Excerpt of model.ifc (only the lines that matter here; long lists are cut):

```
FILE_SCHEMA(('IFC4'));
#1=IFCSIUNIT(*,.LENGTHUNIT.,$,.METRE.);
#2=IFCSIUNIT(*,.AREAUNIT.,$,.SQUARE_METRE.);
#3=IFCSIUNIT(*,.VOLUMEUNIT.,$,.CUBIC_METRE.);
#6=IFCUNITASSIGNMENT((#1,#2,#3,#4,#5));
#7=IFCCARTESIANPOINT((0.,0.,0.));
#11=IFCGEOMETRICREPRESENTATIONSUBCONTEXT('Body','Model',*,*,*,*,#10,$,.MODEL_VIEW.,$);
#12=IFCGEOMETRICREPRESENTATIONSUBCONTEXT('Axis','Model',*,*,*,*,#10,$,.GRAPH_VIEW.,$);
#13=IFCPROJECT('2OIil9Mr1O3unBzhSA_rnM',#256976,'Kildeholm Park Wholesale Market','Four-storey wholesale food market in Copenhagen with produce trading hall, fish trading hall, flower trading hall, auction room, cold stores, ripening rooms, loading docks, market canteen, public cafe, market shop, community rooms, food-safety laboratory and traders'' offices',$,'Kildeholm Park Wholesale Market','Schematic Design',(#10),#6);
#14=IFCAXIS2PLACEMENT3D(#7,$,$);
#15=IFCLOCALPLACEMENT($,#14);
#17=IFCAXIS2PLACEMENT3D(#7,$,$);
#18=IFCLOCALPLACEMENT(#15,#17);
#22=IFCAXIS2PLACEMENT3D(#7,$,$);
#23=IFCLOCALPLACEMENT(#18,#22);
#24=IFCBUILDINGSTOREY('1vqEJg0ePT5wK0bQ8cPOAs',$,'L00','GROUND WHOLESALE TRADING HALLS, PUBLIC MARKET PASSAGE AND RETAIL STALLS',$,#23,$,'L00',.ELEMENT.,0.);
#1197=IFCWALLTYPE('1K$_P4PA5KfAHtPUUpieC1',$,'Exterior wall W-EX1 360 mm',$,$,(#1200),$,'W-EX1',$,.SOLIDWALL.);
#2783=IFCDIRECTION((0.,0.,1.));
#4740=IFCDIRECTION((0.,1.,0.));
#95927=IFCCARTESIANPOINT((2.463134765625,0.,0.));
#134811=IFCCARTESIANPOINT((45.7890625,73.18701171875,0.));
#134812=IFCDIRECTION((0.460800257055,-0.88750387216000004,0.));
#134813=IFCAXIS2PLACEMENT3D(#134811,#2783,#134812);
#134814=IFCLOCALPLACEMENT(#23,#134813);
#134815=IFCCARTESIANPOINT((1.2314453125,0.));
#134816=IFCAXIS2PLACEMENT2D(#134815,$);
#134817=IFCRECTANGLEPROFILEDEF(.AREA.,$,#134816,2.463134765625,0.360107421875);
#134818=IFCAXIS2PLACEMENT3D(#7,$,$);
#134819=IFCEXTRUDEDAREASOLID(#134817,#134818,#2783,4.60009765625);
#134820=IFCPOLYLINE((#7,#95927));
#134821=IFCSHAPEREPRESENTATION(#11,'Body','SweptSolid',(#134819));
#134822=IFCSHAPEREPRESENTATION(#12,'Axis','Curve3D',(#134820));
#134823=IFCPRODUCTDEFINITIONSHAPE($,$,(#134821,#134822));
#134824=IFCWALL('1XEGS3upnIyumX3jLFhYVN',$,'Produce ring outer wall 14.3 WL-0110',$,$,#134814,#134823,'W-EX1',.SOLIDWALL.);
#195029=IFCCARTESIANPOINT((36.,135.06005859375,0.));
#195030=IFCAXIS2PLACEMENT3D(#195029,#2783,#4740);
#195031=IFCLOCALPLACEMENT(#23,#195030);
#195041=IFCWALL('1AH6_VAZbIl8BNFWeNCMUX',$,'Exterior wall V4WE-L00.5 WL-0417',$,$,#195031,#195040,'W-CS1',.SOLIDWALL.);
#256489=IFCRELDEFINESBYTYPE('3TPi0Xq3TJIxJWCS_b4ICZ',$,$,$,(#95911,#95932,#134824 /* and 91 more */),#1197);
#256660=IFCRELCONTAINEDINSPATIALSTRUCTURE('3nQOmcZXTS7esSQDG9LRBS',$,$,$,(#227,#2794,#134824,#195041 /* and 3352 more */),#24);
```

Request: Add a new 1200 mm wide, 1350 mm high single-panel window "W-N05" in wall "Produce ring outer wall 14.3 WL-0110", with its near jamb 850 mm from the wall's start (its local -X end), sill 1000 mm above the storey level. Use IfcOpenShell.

```python
import numpy as np
import ifcopenshell
import ifcopenshell.api.feature
import ifcopenshell.api.geometry
import ifcopenshell.api.root
import ifcopenshell.api.spatial
import ifcopenshell.geom
import ifcopenshell.util.element
import ifcopenshell.util.placement
import ifcopenshell.util.representation
import ifcopenshell.util.shape
import ifcopenshell.util.unit

model = ifcopenshell.open("model.ifc")
unit_scale = ifcopenshell.util.unit.calculate_unit_scale(model)
settings = ifcopenshell.geom.settings()


def volume(element):
    """Net volume in cubic metres, openings subtracted."""
    shape = ifcopenshell.geom.create_shape(settings, element)
    return ifcopenshell.util.shape.get_volume(shape.geometry)


wall = model.by_guid("1XEGS3upnIyumX3jLFhYVN")
storey = ifcopenshell.util.element.get_container(wall, ifc_class="IfcBuildingStorey")
context = ifcopenshell.util.representation.get_context(model, "Model", "Body", "MODEL_VIEW")
before = volume(wall)

width, height, from_end, sill = 1.2, 1.35, 0.85, 1  # metres

# The wall runs along its own X axis, and the end named is its -X end.
wall_shape = ifcopenshell.geom.create_shape(settings, wall)
x, y, z = ifcopenshell.util.shape.get_vertices(wall_shape.geometry).T
start = x.min() + from_end
face, thickness = float(y.min()), float(y.max() - y.min())
wall_matrix = ifcopenshell.util.placement.get_local_placement(wall.ObjectPlacement)
level = ifcopenshell.util.placement.get_local_placement(storey.ObjectPlacement)[2, 3]


def in_wall(x, y):
    """Placement at x, y metres in the wall's axes, at sill height."""
    matrix = wall_matrix.copy()
    matrix[:, 3] = wall_matrix @ np.array([x / unit_scale, y / unit_scale, 0.0, 1.0])
    matrix[2, 3] = level + sill / unit_scale
    return matrix


# Opening: a box that overshoots both wall faces by 50 mm.
opening = ifcopenshell.api.root.create_entity(model, ifc_class="IfcOpeningElement", predefined_type="OPENING")
box = ifcopenshell.api.geometry.add_wall_representation(
    model, context=context, length=width, height=height, thickness=thickness + 0.1
)
ifcopenshell.api.geometry.assign_representation(model, product=opening, representation=box)
ifcopenshell.api.geometry.edit_object_placement(model, product=opening, matrix=in_wall(start, face - 0.05), is_si=False)
ifcopenshell.api.feature.add_feature(model, feature=opening, element=wall)

window = ifcopenshell.api.root.create_entity(model, ifc_class="IfcWindow", name="W-N05", predefined_type="WINDOW")
window.OverallWidth, window.OverallHeight = width / unit_scale, height / unit_scale
window.PartitioningType = "SINGLE_PANEL"
body = ifcopenshell.api.geometry.add_window_representation(
    model,
    context=context,
    overall_width=window.OverallWidth,
    overall_height=window.OverallHeight,
    partition_type="SINGLE_PANEL",
)
ifcopenshell.api.geometry.assign_representation(model, product=window, representation=body)
ifcopenshell.api.spatial.assign_container(model, products=[window], relating_structure=storey)
ifcopenshell.api.feature.add_filling(model, opening=opening, element=window)

# Centre the window in the wall's thickness.
ifcopenshell.api.geometry.edit_object_placement(model, product=window, matrix=in_wall(start, face), is_si=False)
window_shape = ifcopenshell.geom.create_shape(settings, window)
depth = ifcopenshell.util.shape.get_vertices(window_shape.geometry)[:, 1]
offset = face + thickness / 2 - (depth.min() + depth.max()) / 2
ifcopenshell.api.geometry.edit_object_placement(model, product=window, matrix=in_wall(start, offset), is_si=False)

after = volume(wall)

print(f"wall volume {before:.3f} -> {after:.3f} m3")

model.write("model-out.ifc")
```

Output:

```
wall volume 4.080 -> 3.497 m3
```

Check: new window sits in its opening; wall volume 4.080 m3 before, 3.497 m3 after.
